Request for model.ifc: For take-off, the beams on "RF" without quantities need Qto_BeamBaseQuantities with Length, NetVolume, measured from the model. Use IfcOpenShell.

First a look at what the model holds.

```python
import ifcopenshell
import ifcopenshell.util.element
import ifcopenshell.util.unit

model = ifcopenshell.open("model.ifc")
print(model.schema)
for unit_type in ("LENGTHUNIT", "AREAUNIT", "VOLUMEUNIT"):
    print(unit_type, ifcopenshell.util.unit.calculate_unit_scale(model, unit_type))
storey = next(s for s in model.by_type("IfcBuildingStorey") if s.Name == "RF")
beams = [e for e in ifcopenshell.util.element.get_decomposition(storey) if e.is_a("IfcBeam")]
for e in sorted(beams, key=lambda e: e.id()):
    print(e.id(), e.is_a(), e.Name, list(ifcopenshell.util.element.get_psets(e, qtos_only=True)), sep=" | ")
```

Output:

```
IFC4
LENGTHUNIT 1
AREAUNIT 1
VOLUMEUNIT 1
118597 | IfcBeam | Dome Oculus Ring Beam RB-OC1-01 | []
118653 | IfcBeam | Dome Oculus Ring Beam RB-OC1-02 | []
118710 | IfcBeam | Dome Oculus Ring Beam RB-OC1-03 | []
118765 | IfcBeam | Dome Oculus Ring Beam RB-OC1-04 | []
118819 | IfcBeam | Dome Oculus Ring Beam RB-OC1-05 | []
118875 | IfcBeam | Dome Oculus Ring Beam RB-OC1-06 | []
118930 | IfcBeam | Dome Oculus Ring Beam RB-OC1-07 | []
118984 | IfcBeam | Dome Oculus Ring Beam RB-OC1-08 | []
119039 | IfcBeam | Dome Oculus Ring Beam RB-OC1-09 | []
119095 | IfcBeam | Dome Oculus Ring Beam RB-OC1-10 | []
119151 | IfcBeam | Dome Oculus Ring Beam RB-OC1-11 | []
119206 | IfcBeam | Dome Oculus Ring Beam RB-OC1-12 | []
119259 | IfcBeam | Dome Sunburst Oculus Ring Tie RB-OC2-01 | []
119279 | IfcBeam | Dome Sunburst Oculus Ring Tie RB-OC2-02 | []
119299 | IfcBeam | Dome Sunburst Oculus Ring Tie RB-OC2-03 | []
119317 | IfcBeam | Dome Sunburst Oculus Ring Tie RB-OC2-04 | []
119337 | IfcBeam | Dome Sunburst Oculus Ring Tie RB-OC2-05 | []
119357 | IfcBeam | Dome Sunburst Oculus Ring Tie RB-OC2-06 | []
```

```python
import ifcopenshell
import ifcopenshell.api.pset
import ifcopenshell.geom
import ifcopenshell.util.element
import ifcopenshell.util.shape
import ifcopenshell.util.unit

model = ifcopenshell.open("model.ifc")
unit_scale = ifcopenshell.util.unit.calculate_unit_scale(model)
volume_scale = ifcopenshell.util.unit.calculate_unit_scale(model, "VOLUMEUNIT")
settings = ifcopenshell.geom.settings()

storey = next(s for s in model.by_type("IfcBuildingStorey") if s.Name == "RF")
beams = [e for e in ifcopenshell.util.element.get_decomposition(storey) if e.is_a("IfcBeam")]

for e in sorted(beams, key=lambda e: e.id()):
    if ifcopenshell.util.element.get_psets(e, qtos_only=True, should_inherit=False):
        continue
    # Geometry comes back in metres, in the element's own axes.
    shape = ifcopenshell.geom.create_shape(settings, e)
    values = {
        "Length": ifcopenshell.util.shape.get_max_xyz(shape.geometry) / unit_scale,
        "NetVolume": ifcopenshell.util.shape.get_volume(shape.geometry) / volume_scale,
    }
    qto = ifcopenshell.api.pset.add_qto(model, product=e, name="Qto_BeamBaseQuantities")
    ifcopenshell.api.pset.edit_qto(model, qto=qto, properties=values)
    print(e.id(), {k: round(v, 3) for k, v in values.items()})

model.write("model_v2.ifc")
```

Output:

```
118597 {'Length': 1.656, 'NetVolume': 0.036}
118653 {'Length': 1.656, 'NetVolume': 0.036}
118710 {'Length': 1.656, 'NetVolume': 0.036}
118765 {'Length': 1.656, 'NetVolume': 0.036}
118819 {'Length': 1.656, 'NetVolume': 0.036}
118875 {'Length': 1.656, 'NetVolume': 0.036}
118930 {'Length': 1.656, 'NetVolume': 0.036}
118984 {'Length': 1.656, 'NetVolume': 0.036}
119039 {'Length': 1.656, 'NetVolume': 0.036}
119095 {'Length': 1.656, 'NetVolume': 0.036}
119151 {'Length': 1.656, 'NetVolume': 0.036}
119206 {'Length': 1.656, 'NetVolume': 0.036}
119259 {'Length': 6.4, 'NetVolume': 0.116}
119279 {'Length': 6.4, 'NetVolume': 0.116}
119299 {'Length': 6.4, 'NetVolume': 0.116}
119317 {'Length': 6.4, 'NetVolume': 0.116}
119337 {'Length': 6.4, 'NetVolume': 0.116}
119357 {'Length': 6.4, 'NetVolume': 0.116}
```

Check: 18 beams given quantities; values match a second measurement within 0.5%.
